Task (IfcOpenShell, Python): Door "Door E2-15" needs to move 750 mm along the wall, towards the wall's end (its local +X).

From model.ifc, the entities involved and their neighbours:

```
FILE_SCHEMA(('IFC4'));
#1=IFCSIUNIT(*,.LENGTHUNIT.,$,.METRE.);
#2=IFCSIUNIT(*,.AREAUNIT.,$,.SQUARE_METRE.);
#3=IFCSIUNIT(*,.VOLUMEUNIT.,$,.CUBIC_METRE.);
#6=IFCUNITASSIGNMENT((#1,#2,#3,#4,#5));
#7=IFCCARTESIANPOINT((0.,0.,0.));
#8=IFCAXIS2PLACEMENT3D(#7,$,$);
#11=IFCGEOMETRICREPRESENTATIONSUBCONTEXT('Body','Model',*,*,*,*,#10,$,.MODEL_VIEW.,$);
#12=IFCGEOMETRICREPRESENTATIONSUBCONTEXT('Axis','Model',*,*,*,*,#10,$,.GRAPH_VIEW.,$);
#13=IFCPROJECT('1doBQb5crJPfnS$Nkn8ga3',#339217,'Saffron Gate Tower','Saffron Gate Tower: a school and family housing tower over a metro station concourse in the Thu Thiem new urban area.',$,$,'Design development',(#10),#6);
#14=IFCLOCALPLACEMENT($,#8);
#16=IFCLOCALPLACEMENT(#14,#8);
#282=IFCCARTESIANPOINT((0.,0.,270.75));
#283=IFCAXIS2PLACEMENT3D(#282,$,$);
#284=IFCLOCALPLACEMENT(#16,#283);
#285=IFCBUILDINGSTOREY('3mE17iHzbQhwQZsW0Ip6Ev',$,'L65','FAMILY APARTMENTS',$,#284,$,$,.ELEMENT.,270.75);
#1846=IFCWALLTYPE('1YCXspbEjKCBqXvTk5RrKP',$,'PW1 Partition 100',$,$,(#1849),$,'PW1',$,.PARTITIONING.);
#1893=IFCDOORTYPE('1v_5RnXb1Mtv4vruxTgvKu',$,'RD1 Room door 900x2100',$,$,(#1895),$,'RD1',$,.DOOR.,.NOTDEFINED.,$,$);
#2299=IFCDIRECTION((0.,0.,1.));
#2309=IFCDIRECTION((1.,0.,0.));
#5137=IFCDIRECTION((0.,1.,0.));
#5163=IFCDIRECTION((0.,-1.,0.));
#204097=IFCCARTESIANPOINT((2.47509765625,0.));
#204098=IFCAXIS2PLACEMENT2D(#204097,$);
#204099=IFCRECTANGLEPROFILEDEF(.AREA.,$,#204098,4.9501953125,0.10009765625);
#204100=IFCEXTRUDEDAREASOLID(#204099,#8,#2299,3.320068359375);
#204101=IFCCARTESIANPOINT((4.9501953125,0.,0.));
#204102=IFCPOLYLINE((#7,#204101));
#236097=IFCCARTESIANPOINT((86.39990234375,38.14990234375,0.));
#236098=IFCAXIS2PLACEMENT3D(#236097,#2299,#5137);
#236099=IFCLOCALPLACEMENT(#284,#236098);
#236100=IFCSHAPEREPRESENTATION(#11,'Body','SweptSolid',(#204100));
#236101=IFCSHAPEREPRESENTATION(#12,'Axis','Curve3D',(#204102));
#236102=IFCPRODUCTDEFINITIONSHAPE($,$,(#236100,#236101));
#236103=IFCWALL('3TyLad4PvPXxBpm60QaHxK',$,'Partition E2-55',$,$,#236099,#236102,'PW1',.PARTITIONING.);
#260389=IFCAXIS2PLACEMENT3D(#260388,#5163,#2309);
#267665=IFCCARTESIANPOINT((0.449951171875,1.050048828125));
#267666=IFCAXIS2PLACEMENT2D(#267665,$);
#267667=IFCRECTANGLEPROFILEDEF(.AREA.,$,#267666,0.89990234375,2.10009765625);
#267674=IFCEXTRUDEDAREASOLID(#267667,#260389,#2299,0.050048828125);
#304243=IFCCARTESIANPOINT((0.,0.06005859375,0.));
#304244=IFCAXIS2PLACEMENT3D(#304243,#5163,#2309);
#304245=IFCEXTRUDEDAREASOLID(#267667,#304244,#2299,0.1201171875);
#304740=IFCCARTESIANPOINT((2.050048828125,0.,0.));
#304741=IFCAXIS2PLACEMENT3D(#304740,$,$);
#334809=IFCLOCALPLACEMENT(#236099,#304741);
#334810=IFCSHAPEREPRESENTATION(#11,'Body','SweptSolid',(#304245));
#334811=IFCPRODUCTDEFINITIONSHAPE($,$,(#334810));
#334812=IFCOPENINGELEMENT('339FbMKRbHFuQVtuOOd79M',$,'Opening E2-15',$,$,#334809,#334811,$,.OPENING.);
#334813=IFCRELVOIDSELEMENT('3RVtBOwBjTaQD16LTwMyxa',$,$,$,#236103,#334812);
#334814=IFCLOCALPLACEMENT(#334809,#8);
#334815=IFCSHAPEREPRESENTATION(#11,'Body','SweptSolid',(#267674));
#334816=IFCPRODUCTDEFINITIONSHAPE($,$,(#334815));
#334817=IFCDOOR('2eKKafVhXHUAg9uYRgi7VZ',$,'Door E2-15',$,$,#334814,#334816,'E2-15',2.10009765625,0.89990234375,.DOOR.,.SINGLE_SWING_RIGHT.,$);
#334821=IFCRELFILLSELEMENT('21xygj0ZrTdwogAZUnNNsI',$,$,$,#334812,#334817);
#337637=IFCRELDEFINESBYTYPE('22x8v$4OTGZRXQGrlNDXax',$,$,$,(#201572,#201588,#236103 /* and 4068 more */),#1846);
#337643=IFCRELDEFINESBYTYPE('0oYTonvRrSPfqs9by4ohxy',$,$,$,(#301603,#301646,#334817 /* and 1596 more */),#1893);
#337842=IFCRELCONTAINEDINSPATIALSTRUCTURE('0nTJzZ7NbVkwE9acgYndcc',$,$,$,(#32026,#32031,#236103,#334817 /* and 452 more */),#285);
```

```python
import ifcopenshell
import ifcopenshell.api.geometry
import ifcopenshell.util.placement

model = ifcopenshell.open("model.ifc")

door = model.by_id(334817)
opening = door.FillsVoids[0].RelatingOpeningElement
wall = opening.VoidsElements[0].RelatingBuildingElement

wall_matrix = ifcopenshell.util.placement.get_local_placement(wall.ObjectPlacement)
shift = wall_matrix[:3, 0] * 0.75
before = ifcopenshell.util.placement.get_local_placement(door.ObjectPlacement)[:3, 3].copy()

# The door is placed relative to its opening, so it follows when the opening moves.
matrix = ifcopenshell.util.placement.get_local_placement(opening.ObjectPlacement)
matrix[:3, 3] += shift
ifcopenshell.api.geometry.edit_object_placement(
    model, product=opening, matrix=matrix, is_si=False, should_transform_children=True
)

after = ifcopenshell.util.placement.get_local_placement(door.ObjectPlacement)[:3, 3]
print("door moved by", (after - before).round(3) + 0.0)

model.write("model_edited.ifc")
```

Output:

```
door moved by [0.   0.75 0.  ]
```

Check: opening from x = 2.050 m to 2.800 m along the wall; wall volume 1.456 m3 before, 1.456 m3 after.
